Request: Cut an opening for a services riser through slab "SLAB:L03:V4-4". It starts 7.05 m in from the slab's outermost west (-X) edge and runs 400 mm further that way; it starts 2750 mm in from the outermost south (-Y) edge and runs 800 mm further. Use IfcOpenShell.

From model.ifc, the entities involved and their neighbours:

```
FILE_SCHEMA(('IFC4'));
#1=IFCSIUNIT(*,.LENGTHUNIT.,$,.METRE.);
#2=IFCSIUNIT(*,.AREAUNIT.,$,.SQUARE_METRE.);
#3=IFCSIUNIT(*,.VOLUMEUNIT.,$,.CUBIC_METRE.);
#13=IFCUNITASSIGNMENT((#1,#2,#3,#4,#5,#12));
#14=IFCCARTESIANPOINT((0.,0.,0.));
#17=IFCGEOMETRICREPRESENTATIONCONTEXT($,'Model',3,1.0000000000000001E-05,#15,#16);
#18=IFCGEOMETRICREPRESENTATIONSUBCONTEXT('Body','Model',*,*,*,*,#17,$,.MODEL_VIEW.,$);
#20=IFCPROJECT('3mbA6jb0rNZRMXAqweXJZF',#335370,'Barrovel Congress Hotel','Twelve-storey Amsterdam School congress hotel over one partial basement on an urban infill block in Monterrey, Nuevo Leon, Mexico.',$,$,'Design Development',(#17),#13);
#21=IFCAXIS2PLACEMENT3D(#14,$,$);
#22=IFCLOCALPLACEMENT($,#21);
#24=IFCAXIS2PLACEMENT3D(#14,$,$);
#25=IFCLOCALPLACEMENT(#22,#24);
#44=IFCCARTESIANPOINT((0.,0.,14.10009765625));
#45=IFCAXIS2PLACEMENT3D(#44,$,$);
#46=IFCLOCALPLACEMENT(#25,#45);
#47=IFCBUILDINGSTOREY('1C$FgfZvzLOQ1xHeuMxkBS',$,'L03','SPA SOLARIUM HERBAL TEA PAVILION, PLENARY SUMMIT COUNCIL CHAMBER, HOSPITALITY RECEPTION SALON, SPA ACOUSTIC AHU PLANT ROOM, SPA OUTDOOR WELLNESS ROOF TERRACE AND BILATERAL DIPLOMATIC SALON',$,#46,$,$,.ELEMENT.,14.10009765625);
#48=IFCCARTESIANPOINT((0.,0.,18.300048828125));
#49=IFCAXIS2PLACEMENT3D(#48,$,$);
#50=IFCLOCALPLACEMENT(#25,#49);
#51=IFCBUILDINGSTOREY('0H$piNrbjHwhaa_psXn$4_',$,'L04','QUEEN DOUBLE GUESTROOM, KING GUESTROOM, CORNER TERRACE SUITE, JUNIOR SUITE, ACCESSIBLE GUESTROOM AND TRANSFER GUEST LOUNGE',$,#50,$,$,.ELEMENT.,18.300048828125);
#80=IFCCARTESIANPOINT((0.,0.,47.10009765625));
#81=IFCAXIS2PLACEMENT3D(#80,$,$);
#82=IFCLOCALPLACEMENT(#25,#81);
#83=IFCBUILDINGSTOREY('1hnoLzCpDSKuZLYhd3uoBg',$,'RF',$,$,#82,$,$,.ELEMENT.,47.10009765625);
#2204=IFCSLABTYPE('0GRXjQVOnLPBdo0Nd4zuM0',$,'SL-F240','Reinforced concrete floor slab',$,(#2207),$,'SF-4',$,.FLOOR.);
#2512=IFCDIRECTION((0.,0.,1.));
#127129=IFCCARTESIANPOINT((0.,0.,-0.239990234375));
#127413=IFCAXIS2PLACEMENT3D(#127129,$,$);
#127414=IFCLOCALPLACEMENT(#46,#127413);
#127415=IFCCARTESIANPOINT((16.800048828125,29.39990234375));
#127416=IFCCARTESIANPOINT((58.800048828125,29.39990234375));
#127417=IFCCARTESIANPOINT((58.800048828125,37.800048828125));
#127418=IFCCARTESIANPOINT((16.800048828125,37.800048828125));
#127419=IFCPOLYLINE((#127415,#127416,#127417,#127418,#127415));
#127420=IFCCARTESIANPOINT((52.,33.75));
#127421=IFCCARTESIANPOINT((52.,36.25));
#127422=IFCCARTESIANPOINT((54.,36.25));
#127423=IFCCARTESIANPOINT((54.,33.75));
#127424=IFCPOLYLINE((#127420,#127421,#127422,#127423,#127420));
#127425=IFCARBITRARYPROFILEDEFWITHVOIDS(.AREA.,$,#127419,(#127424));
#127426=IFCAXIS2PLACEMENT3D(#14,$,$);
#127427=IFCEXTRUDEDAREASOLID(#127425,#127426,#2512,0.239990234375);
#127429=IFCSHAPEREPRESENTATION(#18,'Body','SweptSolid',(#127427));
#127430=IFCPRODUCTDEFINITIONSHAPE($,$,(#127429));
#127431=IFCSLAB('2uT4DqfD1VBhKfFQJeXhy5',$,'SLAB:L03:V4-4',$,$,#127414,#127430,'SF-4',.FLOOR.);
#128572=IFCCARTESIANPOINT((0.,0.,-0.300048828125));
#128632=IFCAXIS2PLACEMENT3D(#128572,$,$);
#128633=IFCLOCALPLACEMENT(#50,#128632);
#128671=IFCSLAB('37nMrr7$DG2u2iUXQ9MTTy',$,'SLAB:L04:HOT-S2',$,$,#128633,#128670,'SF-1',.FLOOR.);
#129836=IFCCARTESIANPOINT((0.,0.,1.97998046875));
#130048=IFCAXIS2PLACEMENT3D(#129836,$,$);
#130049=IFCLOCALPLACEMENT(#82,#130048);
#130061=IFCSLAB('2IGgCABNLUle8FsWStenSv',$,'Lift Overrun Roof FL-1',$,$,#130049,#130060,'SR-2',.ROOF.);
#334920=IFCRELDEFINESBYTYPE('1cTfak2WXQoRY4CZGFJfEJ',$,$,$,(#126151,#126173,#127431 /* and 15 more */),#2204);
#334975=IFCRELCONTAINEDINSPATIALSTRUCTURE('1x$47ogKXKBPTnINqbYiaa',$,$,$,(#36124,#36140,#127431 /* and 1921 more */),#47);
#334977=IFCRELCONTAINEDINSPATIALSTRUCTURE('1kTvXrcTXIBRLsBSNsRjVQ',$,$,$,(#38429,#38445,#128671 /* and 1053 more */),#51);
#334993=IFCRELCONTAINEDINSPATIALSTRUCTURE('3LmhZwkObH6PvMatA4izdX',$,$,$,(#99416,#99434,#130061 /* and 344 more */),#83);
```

```python
import numpy as np
import ifcopenshell
import ifcopenshell.api.feature
import ifcopenshell.api.geometry
import ifcopenshell.api.root
import ifcopenshell.geom
import ifcopenshell.util.placement
import ifcopenshell.util.representation
import ifcopenshell.util.shape
import ifcopenshell.util.unit

model = ifcopenshell.open("model.ifc")
unit_scale = ifcopenshell.util.unit.calculate_unit_scale(model)
settings = ifcopenshell.geom.settings()


def volume(element):
    """Net volume in cubic metres, openings subtracted."""
    shape = ifcopenshell.geom.create_shape(settings, element)
    return ifcopenshell.util.shape.get_volume(shape.geometry)


slab = model.by_guid("2uT4DqfD1VBhKfFQJeXhy5")
before = volume(slab)

# Extent in the slab's own axes, in metres. The edges named are its -X and -Y sides.
slab_shape = ifcopenshell.geom.create_shape(settings, slab)
vertices = ifcopenshell.util.shape.get_vertices(slab_shape.geometry)
x_min, y_min, bottom = vertices.min(axis=0)
top = vertices[:, 2].max()

opening = ifcopenshell.api.root.create_entity(model, ifc_class="IfcOpeningElement", name="Services riser opening", predefined_type="OPENING")
context = ifcopenshell.util.representation.get_context(model, "Model", "Body", "MODEL_VIEW")
width, depth = 0.4, 0.8
outline = [(0.0, 0.0), (width, 0.0), (width, depth), (0.0, depth), (0.0, 0.0)]
# Overshoot both faces by 50 mm so the cut is clean.
shape = ifcopenshell.api.geometry.add_slab_representation(
    model, context=context, depth=top - bottom + 0.1, polyline=outline
)
ifcopenshell.api.geometry.assign_representation(model, product=opening, representation=shape)

matrix = ifcopenshell.util.placement.get_local_placement(slab.ObjectPlacement)
matrix[:, 3] = matrix @ np.append(np.array([x_min + 7.05, y_min + 2.75, bottom - 0.05]) / unit_scale, 1.0)
ifcopenshell.api.geometry.edit_object_placement(model, product=opening, matrix=matrix, is_si=False)
ifcopenshell.api.feature.add_feature(model, feature=opening, element=slab)

after = volume(slab)

print(f"slab volume {before:.3f} -> {after:.3f} m3")

model.write("model_edited.ifc")
```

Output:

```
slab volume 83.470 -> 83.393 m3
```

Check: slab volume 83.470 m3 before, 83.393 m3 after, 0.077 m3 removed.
